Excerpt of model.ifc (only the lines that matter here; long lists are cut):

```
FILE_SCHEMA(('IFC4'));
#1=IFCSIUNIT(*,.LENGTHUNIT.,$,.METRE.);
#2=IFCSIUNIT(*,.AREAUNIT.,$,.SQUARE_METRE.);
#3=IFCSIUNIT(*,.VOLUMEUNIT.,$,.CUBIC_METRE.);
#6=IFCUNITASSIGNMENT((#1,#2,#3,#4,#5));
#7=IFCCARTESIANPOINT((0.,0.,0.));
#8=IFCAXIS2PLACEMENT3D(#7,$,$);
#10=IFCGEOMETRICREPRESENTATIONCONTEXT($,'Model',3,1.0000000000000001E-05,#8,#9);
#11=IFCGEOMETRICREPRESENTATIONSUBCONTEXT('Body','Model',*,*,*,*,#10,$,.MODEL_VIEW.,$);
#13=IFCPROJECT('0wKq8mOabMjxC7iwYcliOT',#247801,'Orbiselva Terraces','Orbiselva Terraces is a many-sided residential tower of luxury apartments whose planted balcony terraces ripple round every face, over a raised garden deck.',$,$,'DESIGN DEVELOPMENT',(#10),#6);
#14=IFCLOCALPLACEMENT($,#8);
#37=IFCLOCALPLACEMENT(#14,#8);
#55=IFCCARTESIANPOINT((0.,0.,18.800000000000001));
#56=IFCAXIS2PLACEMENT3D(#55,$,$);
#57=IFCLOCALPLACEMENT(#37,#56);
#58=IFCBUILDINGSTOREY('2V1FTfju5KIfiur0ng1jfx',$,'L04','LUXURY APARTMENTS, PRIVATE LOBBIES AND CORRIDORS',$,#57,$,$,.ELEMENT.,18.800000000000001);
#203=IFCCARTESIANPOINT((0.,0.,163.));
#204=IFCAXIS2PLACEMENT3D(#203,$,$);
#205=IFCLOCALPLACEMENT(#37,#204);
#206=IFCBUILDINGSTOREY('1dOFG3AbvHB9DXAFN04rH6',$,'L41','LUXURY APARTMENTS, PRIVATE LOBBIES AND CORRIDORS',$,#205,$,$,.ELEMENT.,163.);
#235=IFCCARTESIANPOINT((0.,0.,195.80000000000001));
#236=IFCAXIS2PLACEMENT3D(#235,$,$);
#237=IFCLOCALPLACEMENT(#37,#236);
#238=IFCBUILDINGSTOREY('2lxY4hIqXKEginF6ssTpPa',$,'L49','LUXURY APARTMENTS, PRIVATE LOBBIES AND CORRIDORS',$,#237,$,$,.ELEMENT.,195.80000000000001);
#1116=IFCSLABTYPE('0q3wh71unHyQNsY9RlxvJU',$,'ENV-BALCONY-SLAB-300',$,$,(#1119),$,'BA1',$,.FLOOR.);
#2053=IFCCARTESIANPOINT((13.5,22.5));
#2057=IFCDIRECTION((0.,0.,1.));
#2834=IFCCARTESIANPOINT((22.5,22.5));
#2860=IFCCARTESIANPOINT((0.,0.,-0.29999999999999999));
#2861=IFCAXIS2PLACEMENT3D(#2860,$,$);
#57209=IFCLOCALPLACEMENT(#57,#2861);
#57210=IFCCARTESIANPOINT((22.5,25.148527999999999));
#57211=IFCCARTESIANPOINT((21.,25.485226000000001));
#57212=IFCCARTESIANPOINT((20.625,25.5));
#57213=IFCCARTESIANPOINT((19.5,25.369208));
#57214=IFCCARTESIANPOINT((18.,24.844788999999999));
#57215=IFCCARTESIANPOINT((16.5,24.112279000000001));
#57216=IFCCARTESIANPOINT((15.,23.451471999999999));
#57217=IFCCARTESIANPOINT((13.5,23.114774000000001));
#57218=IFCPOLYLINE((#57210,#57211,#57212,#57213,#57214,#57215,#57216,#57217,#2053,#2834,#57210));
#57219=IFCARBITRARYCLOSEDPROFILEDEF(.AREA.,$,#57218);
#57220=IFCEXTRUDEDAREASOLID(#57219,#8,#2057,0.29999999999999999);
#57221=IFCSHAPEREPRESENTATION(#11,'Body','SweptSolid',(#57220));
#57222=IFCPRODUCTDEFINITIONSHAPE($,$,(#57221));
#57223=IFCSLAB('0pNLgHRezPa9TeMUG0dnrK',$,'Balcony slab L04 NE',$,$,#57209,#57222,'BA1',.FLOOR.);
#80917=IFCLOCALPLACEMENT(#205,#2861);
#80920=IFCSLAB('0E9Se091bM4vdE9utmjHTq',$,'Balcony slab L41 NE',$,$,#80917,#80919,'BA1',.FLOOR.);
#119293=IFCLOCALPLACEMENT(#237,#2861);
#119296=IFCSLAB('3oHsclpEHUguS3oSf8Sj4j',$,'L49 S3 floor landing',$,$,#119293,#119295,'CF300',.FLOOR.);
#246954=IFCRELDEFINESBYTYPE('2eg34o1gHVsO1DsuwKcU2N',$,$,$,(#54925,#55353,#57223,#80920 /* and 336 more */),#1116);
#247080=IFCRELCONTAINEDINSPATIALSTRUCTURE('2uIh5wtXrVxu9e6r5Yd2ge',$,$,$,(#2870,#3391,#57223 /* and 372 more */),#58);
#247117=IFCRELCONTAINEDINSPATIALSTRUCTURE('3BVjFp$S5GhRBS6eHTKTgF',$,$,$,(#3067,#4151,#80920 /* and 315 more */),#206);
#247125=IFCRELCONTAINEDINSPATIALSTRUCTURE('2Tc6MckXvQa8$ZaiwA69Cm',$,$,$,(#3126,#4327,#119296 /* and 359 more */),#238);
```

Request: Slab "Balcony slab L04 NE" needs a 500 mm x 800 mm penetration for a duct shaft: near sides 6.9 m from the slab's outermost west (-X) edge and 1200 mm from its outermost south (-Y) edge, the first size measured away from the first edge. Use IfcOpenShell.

```python
import numpy as np
import ifcopenshell
import ifcopenshell.api.feature
import ifcopenshell.api.geometry
import ifcopenshell.api.root
import ifcopenshell.geom
import ifcopenshell.util.placement
import ifcopenshell.util.representation
import ifcopenshell.util.shape
import ifcopenshell.util.unit

model = ifcopenshell.open("model.ifc")
unit_scale = ifcopenshell.util.unit.calculate_unit_scale(model)
settings = ifcopenshell.geom.settings()


def volume(element):
    """Net volume in cubic metres, openings subtracted."""
    shape = ifcopenshell.geom.create_shape(settings, element)
    return ifcopenshell.util.shape.get_volume(shape.geometry)


slab = model.by_guid("0pNLgHRezPa9TeMUG0dnrK")
before = volume(slab)

# Extent in the slab's own axes, in metres. The edges named are its -X and -Y sides.
slab_shape = ifcopenshell.geom.create_shape(settings, slab)
vertices = ifcopenshell.util.shape.get_vertices(slab_shape.geometry)
x_min, y_min, bottom = vertices.min(axis=0)
top = vertices[:, 2].max()

opening = ifcopenshell.api.root.create_entity(model, ifc_class="IfcOpeningElement", name="Duct shaft opening", predefined_type="OPENING")
context = ifcopenshell.util.representation.get_context(model, "Model", "Body", "MODEL_VIEW")
width, depth = 0.5, 0.8
outline = [(0.0, 0.0), (width, 0.0), (width, depth), (0.0, depth), (0.0, 0.0)]
# Overshoot both faces by 50 mm so the cut is clean.
shape = ifcopenshell.api.geometry.add_slab_representation(
    model, context=context, depth=top - bottom + 0.1, polyline=outline
)
ifcopenshell.api.geometry.assign_representation(model, product=opening, representation=shape)

matrix = ifcopenshell.util.placement.get_local_placement(slab.ObjectPlacement)
matrix[:, 3] = matrix @ np.append(np.array([x_min + 6.9, y_min + 1.2, bottom - 0.05]) / unit_scale, 1.0)
ifcopenshell.api.geometry.edit_object_placement(model, product=opening, matrix=matrix, is_si=False)
ifcopenshell.api.feature.add_feature(model, feature=opening, element=slab)

after = volume(slab)

print(f"slab volume {before:.3f} -> {after:.3f} m3")

model.write("model_rev.ifc")
```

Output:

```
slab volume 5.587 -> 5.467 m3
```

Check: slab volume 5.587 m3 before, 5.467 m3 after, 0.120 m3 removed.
